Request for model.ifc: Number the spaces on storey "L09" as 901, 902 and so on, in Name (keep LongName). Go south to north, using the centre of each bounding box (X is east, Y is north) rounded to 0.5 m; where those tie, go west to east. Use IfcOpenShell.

First a look at what the model holds.

```python
import ifcopenshell
import ifcopenshell.util.element
import ifcopenshell.util.placement

model = ifcopenshell.open("model.ifc")
print(model.schema)
storey = next(s for s in model.by_type("IfcBuildingStorey") if s.Name == "L09")
spaces = [e for e in ifcopenshell.util.element.get_decomposition(storey) if e.is_a("IfcSpace")]
for e in sorted(spaces, key=lambda e: e.id()):
    origin = ifcopenshell.util.placement.get_local_placement(e.ObjectPlacement)[:3, 3]
    print(e.id(), e.Name, e.LongName, origin.round(2) + 0.0, sep=" | ")
```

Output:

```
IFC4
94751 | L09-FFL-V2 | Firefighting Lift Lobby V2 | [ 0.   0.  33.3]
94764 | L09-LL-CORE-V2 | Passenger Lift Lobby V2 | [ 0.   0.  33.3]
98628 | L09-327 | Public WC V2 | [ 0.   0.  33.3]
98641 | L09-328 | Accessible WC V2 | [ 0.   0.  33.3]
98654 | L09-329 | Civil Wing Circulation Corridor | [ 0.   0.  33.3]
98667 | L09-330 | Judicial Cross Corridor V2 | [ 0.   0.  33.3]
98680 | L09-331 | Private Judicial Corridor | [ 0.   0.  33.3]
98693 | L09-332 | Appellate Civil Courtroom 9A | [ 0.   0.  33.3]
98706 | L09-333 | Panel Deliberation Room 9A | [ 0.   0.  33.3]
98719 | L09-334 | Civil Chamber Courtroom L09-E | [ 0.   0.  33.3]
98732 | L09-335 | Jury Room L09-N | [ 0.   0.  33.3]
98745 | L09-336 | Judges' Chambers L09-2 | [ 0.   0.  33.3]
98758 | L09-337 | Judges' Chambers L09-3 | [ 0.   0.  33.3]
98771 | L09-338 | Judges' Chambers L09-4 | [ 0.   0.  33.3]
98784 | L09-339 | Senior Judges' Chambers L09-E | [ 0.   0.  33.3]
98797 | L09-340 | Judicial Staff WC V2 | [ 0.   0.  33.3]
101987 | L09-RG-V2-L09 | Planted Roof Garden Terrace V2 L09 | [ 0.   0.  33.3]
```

```python
import ifcopenshell
import ifcopenshell.geom
import ifcopenshell.util.element
import ifcopenshell.util.shape

model = ifcopenshell.open("model.ifc")
settings = ifcopenshell.geom.settings()
settings.set("use-world-coords", True)


def centre(element):
    shape = ifcopenshell.geom.create_shape(settings, element)
    return ifcopenshell.util.shape.get_bbox_centroid(shape.geometry)


storey = next(s for s in model.by_type("IfcBuildingStorey") if s.Name == "L09")
spaces = [e for e in ifcopenshell.util.element.get_decomposition(storey) if e.is_a("IfcSpace")]

# Insertion points can sit at a corner or the storey origin, so sort by the geometry (in metres).
centres = {e: centre(e) for e in spaces}
spaces.sort(key=lambda e: (round(centres[e][1] / 0.5), centres[e][0]))

for i, e in enumerate(spaces, start=1):
    number = f"9{i:02d}"
    e.Name = number
    print(e.id(), number)

model.write("model_rev.ifc")
```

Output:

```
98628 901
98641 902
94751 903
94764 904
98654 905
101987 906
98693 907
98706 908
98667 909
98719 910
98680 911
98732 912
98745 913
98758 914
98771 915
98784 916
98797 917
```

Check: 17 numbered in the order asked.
